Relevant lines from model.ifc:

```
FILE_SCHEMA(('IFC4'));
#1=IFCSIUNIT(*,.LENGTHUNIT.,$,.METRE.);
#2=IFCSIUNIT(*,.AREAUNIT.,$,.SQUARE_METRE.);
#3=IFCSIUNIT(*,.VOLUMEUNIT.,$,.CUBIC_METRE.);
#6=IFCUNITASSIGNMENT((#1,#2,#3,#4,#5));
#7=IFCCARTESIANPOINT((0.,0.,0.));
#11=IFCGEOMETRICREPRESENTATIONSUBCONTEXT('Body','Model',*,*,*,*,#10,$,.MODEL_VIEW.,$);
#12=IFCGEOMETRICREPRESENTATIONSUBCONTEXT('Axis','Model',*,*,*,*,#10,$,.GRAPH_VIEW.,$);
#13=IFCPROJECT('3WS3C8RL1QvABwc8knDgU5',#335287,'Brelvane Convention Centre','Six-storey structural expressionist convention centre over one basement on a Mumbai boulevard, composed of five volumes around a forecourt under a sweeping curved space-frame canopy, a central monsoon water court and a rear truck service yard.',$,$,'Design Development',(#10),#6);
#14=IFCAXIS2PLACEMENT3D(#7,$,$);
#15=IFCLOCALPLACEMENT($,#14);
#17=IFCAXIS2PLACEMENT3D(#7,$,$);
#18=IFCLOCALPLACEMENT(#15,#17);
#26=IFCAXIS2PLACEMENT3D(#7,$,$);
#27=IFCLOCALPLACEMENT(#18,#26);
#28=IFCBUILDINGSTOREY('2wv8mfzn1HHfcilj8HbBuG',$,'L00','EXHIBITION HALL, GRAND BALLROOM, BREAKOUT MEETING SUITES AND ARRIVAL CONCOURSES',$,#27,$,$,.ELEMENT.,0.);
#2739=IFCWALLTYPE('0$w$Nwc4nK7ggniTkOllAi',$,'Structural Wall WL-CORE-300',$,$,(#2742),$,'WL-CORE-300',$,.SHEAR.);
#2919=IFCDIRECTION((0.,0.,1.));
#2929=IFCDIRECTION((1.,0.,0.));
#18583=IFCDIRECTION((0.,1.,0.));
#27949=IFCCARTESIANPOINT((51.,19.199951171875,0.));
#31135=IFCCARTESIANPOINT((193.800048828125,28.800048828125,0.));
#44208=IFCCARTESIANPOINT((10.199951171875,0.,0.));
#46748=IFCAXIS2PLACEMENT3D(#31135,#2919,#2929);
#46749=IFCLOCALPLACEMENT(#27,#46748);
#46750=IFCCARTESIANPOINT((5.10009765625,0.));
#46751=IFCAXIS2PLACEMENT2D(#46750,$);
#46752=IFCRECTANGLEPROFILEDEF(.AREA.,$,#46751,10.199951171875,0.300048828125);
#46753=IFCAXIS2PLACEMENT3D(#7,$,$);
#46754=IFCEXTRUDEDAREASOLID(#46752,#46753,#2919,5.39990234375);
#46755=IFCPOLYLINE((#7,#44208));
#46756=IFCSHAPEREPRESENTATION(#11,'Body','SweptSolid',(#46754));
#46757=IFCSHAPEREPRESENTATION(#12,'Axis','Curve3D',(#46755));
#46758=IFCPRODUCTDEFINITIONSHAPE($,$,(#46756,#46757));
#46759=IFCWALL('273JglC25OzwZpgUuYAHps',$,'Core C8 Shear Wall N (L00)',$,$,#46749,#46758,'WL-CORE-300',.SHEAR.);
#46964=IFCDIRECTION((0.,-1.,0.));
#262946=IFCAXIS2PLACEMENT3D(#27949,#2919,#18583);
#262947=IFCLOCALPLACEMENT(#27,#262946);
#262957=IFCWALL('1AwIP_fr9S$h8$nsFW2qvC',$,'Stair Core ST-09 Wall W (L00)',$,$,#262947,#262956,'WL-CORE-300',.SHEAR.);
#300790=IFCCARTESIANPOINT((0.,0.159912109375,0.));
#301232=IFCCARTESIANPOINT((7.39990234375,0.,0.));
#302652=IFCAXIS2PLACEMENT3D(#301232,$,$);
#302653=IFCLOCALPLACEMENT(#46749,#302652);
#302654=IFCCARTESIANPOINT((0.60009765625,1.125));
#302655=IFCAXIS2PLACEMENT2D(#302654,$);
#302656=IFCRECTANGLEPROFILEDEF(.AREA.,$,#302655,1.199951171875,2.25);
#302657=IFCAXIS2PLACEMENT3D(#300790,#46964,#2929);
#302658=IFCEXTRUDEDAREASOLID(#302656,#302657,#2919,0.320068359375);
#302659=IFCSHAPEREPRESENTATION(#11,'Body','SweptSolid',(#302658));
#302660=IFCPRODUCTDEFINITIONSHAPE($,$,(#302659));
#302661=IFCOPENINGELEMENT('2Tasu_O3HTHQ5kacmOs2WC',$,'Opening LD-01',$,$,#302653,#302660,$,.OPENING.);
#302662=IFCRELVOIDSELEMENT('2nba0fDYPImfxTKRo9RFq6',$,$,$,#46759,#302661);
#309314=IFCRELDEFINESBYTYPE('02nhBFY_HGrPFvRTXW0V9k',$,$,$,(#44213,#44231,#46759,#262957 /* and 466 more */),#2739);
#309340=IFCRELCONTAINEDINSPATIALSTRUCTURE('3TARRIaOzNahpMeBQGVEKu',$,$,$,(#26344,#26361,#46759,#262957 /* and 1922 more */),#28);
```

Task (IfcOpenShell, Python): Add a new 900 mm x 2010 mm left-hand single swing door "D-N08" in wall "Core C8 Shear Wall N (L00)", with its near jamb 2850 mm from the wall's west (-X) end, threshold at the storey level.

```python
import numpy as np
import ifcopenshell
import ifcopenshell.api.feature
import ifcopenshell.api.geometry
import ifcopenshell.api.root
import ifcopenshell.api.spatial
import ifcopenshell.geom
import ifcopenshell.util.element
import ifcopenshell.util.placement
import ifcopenshell.util.representation
import ifcopenshell.util.shape
import ifcopenshell.util.unit

model = ifcopenshell.open("model.ifc")
unit_scale = ifcopenshell.util.unit.calculate_unit_scale(model)
settings = ifcopenshell.geom.settings()


def volume(element):
    """Net volume in cubic metres, openings subtracted."""
    shape = ifcopenshell.geom.create_shape(settings, element)
    return ifcopenshell.util.shape.get_volume(shape.geometry)


wall = model.by_guid("273JglC25OzwZpgUuYAHps")
storey = ifcopenshell.util.element.get_container(wall, ifc_class="IfcBuildingStorey")
context = ifcopenshell.util.representation.get_context(model, "Model", "Body", "MODEL_VIEW")
before = volume(wall)

width, height, from_end, sill = 0.9, 2.01, 2.85, 0.0  # metres

# The wall runs along its own X axis, and the end named is its -X end.
wall_shape = ifcopenshell.geom.create_shape(settings, wall)
x, y, z = ifcopenshell.util.shape.get_vertices(wall_shape.geometry).T
start = x.min() + from_end
face, thickness = float(y.min()), float(y.max() - y.min())
wall_matrix = ifcopenshell.util.placement.get_local_placement(wall.ObjectPlacement)
level = ifcopenshell.util.placement.get_local_placement(storey.ObjectPlacement)[2, 3]


def in_wall(x, y):
    """Placement at x, y metres in the wall's axes, at sill height."""
    matrix = wall_matrix.copy()
    matrix[:, 3] = wall_matrix @ np.array([x / unit_scale, y / unit_scale, 0.0, 1.0])
    matrix[2, 3] = level + sill / unit_scale
    return matrix


# Opening: a box that overshoots both wall faces by 50 mm.
opening = ifcopenshell.api.root.create_entity(model, ifc_class="IfcOpeningElement", predefined_type="OPENING")
box = ifcopenshell.api.geometry.add_wall_representation(
    model, context=context, length=width, height=height, thickness=thickness + 0.1
)
ifcopenshell.api.geometry.assign_representation(model, product=opening, representation=box)
ifcopenshell.api.geometry.edit_object_placement(model, product=opening, matrix=in_wall(start, face - 0.05), is_si=False)
ifcopenshell.api.feature.add_feature(model, feature=opening, element=wall)

door = ifcopenshell.api.root.create_entity(model, ifc_class="IfcDoor", name="D-N08", predefined_type="DOOR")
door.OverallWidth, door.OverallHeight = width / unit_scale, height / unit_scale
door.OperationType = "SINGLE_SWING_LEFT"
body = ifcopenshell.api.geometry.add_door_representation(
    model,
    context=context,
    overall_width=door.OverallWidth,
    overall_height=door.OverallHeight,
    operation_type="SINGLE_SWING_LEFT",
    lining_properties={"LiningDepth": thickness / unit_scale, "ThresholdDepth": thickness / unit_scale},
)
ifcopenshell.api.geometry.assign_representation(model, product=door, representation=body)
ifcopenshell.api.spatial.assign_container(model, products=[door], relating_structure=storey)
ifcopenshell.api.feature.add_filling(model, opening=opening, element=door)

# The lining spans the wall, so the door starts at the wall face.
ifcopenshell.api.geometry.edit_object_placement(model, product=door, matrix=in_wall(start, face), is_si=False)

after = volume(wall)

print(f"wall volume {before:.3f} -> {after:.3f} m3")

model.write("model-out.ifc")
```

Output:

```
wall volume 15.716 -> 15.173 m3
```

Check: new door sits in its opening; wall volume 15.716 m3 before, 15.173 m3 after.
